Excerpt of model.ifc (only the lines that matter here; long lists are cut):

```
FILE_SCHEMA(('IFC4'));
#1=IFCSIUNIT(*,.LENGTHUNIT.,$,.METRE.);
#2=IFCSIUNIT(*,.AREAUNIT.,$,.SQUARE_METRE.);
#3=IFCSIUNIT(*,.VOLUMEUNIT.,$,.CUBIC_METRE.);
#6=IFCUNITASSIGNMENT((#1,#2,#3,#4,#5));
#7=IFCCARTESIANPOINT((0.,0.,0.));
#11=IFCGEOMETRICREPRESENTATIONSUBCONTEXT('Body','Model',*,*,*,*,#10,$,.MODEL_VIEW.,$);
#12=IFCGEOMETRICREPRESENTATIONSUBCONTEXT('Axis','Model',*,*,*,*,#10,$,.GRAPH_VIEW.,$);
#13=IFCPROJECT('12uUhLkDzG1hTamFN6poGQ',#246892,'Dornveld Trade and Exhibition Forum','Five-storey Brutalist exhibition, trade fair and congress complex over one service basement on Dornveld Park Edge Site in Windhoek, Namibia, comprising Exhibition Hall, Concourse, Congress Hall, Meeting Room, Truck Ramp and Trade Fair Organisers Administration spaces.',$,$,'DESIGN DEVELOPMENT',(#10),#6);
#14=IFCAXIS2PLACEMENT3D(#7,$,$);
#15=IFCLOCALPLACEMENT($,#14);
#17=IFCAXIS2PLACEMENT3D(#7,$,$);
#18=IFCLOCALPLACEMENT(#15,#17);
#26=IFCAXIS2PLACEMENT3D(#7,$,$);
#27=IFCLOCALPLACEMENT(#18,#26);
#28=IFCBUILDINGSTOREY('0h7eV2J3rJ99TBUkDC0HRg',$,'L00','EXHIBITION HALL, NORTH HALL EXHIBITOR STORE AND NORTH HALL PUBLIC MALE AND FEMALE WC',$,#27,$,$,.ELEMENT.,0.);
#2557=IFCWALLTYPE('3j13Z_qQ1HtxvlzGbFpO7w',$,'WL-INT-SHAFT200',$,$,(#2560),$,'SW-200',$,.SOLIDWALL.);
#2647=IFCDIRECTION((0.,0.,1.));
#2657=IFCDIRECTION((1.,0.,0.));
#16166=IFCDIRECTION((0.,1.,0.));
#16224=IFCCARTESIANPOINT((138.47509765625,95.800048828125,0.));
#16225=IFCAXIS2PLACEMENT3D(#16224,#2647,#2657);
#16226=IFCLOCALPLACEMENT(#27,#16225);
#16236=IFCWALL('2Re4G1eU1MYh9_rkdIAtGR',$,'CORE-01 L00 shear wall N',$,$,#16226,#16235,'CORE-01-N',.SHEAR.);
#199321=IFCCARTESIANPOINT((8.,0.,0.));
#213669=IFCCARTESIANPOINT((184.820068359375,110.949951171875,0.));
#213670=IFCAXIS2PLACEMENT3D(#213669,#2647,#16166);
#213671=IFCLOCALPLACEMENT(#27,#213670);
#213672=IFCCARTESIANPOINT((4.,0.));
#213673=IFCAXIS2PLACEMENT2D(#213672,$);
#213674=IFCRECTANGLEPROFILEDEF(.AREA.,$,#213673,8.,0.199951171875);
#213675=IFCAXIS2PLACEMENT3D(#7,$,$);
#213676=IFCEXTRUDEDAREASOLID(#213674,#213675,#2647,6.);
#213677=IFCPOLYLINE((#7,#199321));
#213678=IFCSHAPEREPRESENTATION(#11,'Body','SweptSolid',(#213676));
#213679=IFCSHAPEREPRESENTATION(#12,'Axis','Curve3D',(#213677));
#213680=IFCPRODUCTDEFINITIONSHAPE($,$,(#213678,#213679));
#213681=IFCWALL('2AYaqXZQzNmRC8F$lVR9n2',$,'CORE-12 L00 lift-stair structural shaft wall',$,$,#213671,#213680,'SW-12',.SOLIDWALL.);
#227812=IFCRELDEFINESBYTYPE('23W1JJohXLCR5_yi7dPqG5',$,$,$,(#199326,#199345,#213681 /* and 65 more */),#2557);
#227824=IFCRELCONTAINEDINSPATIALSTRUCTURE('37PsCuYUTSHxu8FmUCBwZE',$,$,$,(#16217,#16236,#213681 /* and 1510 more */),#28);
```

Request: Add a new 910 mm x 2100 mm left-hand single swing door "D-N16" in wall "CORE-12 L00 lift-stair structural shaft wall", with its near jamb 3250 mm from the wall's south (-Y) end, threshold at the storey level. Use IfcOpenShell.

```python
import numpy as np
import ifcopenshell
import ifcopenshell.api.feature
import ifcopenshell.api.geometry
import ifcopenshell.api.root
import ifcopenshell.api.spatial
import ifcopenshell.geom
import ifcopenshell.util.element
import ifcopenshell.util.placement
import ifcopenshell.util.representation
import ifcopenshell.util.shape
import ifcopenshell.util.unit

model = ifcopenshell.open("model.ifc")
unit_scale = ifcopenshell.util.unit.calculate_unit_scale(model)
settings = ifcopenshell.geom.settings()


def volume(element):
    """Net volume in cubic metres, openings subtracted."""
    shape = ifcopenshell.geom.create_shape(settings, element)
    return ifcopenshell.util.shape.get_volume(shape.geometry)


wall = model.by_guid("2AYaqXZQzNmRC8F$lVR9n2")
storey = ifcopenshell.util.element.get_container(wall, ifc_class="IfcBuildingStorey")
context = ifcopenshell.util.representation.get_context(model, "Model", "Body", "MODEL_VIEW")
before = volume(wall)

width, height, from_end, sill = 0.91, 2.1, 3.25, 0.0  # metres

# The wall runs along its own X axis, and the end named is its -X end.
wall_shape = ifcopenshell.geom.create_shape(settings, wall)
x, y, z = ifcopenshell.util.shape.get_vertices(wall_shape.geometry).T
start = x.min() + from_end
face, thickness = float(y.min()), float(y.max() - y.min())
wall_matrix = ifcopenshell.util.placement.get_local_placement(wall.ObjectPlacement)
level = ifcopenshell.util.placement.get_local_placement(storey.ObjectPlacement)[2, 3]


def in_wall(x, y):
    """Placement at x, y metres in the wall's axes, at sill height."""
    matrix = wall_matrix.copy()
    matrix[:, 3] = wall_matrix @ np.array([x / unit_scale, y / unit_scale, 0.0, 1.0])
    matrix[2, 3] = level + sill / unit_scale
    return matrix


# Opening: a box that overshoots both wall faces by 50 mm.
opening = ifcopenshell.api.root.create_entity(model, ifc_class="IfcOpeningElement", predefined_type="OPENING")
box = ifcopenshell.api.geometry.add_wall_representation(
    model, context=context, length=width, height=height, thickness=thickness + 0.1
)
ifcopenshell.api.geometry.assign_representation(model, product=opening, representation=box)
ifcopenshell.api.geometry.edit_object_placement(model, product=opening, matrix=in_wall(start, face - 0.05), is_si=False)
ifcopenshell.api.feature.add_feature(model, feature=opening, element=wall)

door = ifcopenshell.api.root.create_entity(model, ifc_class="IfcDoor", name="D-N16", predefined_type="DOOR")
door.OverallWidth, door.OverallHeight = width / unit_scale, height / unit_scale
door.OperationType = "SINGLE_SWING_LEFT"
body = ifcopenshell.api.geometry.add_door_representation(
    model,
    context=context,
    overall_width=door.OverallWidth,
    overall_height=door.OverallHeight,
    operation_type="SINGLE_SWING_LEFT",
    lining_properties={"LiningDepth": thickness / unit_scale, "ThresholdDepth": thickness / unit_scale},
)
ifcopenshell.api.geometry.assign_representation(model, product=door, representation=body)
ifcopenshell.api.spatial.assign_container(model, products=[door], relating_structure=storey)
ifcopenshell.api.feature.add_filling(model, opening=opening, element=door)

# The lining spans the wall, so the door starts at the wall face.
ifcopenshell.api.geometry.edit_object_placement(model, product=door, matrix=in_wall(start, face), is_si=False)

after = volume(wall)

print(f"wall volume {before:.3f} -> {after:.3f} m3")

model.write("model_edited.ifc")
```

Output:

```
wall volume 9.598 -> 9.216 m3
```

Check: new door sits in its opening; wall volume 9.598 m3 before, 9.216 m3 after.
